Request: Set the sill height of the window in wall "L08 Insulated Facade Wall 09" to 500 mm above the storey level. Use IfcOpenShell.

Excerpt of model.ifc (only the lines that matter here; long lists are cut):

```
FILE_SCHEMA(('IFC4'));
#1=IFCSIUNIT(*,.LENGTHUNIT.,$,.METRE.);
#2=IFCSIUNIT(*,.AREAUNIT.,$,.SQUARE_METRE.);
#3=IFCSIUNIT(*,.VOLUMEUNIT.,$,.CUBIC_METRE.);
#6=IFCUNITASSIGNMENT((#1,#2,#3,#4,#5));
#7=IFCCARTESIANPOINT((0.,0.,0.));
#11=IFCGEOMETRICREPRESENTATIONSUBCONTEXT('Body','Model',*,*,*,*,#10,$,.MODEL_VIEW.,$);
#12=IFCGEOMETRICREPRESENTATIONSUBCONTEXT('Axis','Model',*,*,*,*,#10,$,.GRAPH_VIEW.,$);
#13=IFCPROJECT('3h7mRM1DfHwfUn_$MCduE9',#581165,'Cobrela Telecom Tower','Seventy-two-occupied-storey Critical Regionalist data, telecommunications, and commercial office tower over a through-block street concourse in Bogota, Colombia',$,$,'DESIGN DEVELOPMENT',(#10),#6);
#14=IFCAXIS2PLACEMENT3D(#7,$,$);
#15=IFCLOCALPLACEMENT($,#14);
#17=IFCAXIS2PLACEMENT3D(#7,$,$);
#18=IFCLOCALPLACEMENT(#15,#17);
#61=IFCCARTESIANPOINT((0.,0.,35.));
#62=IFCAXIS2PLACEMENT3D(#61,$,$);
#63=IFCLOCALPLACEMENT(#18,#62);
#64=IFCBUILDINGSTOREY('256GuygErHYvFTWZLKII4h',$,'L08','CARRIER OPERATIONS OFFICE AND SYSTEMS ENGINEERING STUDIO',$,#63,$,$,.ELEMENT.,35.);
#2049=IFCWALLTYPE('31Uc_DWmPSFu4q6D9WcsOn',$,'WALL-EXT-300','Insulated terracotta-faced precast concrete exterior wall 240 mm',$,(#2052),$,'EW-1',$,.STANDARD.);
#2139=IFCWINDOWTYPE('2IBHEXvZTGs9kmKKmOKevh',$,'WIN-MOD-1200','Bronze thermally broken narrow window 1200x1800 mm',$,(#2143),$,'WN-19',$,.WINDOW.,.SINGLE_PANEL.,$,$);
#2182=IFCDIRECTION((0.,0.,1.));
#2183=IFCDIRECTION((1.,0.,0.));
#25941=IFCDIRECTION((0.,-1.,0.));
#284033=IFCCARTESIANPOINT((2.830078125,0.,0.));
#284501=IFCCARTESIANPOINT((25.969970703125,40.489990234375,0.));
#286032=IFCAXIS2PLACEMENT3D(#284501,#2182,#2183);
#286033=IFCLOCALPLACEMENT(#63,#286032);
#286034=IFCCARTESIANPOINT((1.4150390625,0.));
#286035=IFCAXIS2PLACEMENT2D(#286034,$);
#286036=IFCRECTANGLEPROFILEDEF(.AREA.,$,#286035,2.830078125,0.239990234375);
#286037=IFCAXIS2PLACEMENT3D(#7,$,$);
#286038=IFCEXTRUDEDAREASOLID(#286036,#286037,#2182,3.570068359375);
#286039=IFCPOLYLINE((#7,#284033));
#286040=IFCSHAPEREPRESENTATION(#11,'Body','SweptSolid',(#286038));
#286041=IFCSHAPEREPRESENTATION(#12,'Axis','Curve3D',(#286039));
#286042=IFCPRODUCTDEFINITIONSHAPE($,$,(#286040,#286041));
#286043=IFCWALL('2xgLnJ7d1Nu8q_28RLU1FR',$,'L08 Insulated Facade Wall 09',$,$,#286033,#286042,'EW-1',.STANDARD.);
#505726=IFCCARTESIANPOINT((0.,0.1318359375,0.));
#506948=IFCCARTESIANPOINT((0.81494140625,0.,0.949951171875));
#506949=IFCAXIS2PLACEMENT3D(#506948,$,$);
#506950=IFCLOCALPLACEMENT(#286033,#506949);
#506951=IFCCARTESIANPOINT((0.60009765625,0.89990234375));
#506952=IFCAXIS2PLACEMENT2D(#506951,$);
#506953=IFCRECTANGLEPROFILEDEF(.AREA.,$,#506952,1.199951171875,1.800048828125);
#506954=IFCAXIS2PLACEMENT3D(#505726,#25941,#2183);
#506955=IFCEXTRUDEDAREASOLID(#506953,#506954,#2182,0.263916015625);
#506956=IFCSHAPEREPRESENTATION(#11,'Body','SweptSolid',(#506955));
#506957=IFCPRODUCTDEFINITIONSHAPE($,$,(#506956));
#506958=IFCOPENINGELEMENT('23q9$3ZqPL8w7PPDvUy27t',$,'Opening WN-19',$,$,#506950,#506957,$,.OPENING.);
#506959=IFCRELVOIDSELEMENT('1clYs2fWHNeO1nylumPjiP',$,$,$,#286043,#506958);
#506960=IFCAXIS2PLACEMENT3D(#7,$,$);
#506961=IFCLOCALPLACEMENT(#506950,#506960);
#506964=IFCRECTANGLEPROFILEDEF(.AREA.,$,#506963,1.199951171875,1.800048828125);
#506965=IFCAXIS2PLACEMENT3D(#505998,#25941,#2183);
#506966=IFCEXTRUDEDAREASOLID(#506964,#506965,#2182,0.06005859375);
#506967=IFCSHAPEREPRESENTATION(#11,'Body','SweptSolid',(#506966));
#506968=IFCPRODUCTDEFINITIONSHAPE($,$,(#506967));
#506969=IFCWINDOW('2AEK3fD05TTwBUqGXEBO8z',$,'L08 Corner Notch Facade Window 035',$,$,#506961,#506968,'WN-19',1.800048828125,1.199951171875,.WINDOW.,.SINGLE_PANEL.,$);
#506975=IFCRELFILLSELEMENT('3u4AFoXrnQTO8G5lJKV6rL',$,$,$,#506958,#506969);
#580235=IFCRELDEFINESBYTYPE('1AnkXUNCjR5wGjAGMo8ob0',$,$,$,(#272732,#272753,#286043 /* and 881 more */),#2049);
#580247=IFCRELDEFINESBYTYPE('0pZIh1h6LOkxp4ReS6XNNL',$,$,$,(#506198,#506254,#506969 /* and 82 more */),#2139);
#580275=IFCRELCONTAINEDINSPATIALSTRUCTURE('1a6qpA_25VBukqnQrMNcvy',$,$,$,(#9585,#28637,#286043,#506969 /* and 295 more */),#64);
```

```python
import numpy as np
import ifcopenshell
import ifcopenshell.api.geometry
import ifcopenshell.geom
import ifcopenshell.util.element
import ifcopenshell.util.placement
import ifcopenshell.util.shape
import ifcopenshell.util.unit

model = ifcopenshell.open("model.ifc")
unit_scale = ifcopenshell.util.unit.calculate_unit_scale(model)

window = model.by_guid("2AEK3fD05TTwBUqGXEBO8z")
opening = window.FillsVoids[0].RelatingOpeningElement
storey = ifcopenshell.util.element.get_container(window, ifc_class="IfcBuildingStorey")
level = ifcopenshell.util.placement.get_local_placement(storey.ObjectPlacement)[2, 3]

# The opening's origin need not be at the sill, so measure its lowest point.
shape = ifcopenshell.geom.create_shape(ifcopenshell.geom.settings(), opening)
bottom = ifcopenshell.util.shape.get_shape_bottom_elevation(shape, shape.geometry) / unit_scale
dz = level + 0.5 / unit_scale - bottom

shift = np.array([0.0, 0.0, dz])
# The window is placed relative to its opening, so it follows when the opening moves.
matrix = ifcopenshell.util.placement.get_local_placement(opening.ObjectPlacement)
matrix[:3, 3] += shift
ifcopenshell.api.geometry.edit_object_placement(
    model, product=opening, matrix=matrix, is_si=False, should_transform_children=True
)

print(f"moved by {dz * unit_scale:+.3f} m")

model.write("model-out.ifc")
```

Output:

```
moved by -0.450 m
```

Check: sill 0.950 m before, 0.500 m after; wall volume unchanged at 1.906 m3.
